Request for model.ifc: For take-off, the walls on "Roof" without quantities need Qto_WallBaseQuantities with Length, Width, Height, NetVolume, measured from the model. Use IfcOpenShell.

First a look at what the model holds.

```python
import ifcopenshell
import ifcopenshell.util.element
import ifcopenshell.util.unit

model = ifcopenshell.open("model.ifc")
print(model.schema)
for unit_type in ("LENGTHUNIT", "AREAUNIT", "VOLUMEUNIT"):
    print(unit_type, ifcopenshell.util.unit.calculate_unit_scale(model, unit_type))
storey = next(s for s in model.by_type("IfcBuildingStorey") if s.Name == "Roof")
walls = [e for e in ifcopenshell.util.element.get_decomposition(storey) if e.is_a("IfcWall")]
for e in sorted(walls, key=lambda e: e.id()):
    print(e.id(), e.is_a(), e.Name, list(ifcopenshell.util.element.get_psets(e, qtos_only=True)), sep=" | ")
```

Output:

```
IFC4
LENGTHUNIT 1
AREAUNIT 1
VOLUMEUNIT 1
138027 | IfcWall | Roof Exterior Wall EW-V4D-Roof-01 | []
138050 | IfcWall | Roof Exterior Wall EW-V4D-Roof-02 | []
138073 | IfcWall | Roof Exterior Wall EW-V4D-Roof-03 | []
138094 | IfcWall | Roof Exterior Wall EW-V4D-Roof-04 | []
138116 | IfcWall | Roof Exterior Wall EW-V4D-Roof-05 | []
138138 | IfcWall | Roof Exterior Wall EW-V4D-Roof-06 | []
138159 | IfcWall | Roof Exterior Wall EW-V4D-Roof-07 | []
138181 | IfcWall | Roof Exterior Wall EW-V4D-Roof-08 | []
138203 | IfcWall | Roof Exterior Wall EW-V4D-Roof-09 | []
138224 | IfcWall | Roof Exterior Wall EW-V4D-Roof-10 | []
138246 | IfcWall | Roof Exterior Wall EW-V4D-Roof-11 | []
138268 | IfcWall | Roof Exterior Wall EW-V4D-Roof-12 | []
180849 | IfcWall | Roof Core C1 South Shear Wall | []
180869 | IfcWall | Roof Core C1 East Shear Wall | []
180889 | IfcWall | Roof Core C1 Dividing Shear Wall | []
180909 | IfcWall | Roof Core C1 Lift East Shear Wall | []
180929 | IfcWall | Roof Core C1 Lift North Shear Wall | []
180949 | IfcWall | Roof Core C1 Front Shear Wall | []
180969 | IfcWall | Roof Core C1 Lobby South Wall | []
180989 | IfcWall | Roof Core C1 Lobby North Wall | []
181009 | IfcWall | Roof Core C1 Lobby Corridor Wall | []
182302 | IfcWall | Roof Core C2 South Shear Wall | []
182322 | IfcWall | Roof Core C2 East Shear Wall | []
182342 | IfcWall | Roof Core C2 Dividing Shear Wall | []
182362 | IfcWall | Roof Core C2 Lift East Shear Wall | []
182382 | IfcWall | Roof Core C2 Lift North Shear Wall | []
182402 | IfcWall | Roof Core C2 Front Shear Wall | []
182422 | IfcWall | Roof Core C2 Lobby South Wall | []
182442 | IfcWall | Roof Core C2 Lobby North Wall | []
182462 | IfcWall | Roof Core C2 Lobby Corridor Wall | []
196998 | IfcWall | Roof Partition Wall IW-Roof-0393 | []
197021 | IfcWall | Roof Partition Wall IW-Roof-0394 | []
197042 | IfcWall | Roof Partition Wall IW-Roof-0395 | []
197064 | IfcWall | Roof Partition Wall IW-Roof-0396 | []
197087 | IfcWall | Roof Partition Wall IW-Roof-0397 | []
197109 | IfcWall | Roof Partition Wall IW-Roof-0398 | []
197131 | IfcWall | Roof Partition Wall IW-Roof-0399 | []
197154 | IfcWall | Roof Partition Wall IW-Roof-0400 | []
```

```python
import ifcopenshell
import ifcopenshell.api.pset
import ifcopenshell.geom
import ifcopenshell.util.element
import ifcopenshell.util.shape
import ifcopenshell.util.unit

model = ifcopenshell.open("model.ifc")
unit_scale = ifcopenshell.util.unit.calculate_unit_scale(model)
volume_scale = ifcopenshell.util.unit.calculate_unit_scale(model, "VOLUMEUNIT")
settings = ifcopenshell.geom.settings()

storey = next(s for s in model.by_type("IfcBuildingStorey") if s.Name == "Roof")
walls = [e for e in ifcopenshell.util.element.get_decomposition(storey) if e.is_a("IfcWall")]

for e in sorted(walls, key=lambda e: e.id()):
    if ifcopenshell.util.element.get_psets(e, qtos_only=True, should_inherit=False):
        continue
    # Geometry comes back in metres, in the element's own axes.
    shape = ifcopenshell.geom.create_shape(settings, e)
    values = {
        "Length": ifcopenshell.util.shape.get_x(shape.geometry) / unit_scale,
        "Width": ifcopenshell.util.shape.get_y(shape.geometry) / unit_scale,
        "Height": ifcopenshell.util.shape.get_z(shape.geometry) / unit_scale,
        "NetVolume": ifcopenshell.util.shape.get_volume(shape.geometry) / volume_scale,
    }
    qto = ifcopenshell.api.pset.add_qto(model, product=e, name="Qto_WallBaseQuantities")
    ifcopenshell.api.pset.edit_qto(model, qto=qto, properties=values)
    print(e.id(), {k: round(v, 3) for k, v in values.items()})

model.write("model_v2.ifc")
```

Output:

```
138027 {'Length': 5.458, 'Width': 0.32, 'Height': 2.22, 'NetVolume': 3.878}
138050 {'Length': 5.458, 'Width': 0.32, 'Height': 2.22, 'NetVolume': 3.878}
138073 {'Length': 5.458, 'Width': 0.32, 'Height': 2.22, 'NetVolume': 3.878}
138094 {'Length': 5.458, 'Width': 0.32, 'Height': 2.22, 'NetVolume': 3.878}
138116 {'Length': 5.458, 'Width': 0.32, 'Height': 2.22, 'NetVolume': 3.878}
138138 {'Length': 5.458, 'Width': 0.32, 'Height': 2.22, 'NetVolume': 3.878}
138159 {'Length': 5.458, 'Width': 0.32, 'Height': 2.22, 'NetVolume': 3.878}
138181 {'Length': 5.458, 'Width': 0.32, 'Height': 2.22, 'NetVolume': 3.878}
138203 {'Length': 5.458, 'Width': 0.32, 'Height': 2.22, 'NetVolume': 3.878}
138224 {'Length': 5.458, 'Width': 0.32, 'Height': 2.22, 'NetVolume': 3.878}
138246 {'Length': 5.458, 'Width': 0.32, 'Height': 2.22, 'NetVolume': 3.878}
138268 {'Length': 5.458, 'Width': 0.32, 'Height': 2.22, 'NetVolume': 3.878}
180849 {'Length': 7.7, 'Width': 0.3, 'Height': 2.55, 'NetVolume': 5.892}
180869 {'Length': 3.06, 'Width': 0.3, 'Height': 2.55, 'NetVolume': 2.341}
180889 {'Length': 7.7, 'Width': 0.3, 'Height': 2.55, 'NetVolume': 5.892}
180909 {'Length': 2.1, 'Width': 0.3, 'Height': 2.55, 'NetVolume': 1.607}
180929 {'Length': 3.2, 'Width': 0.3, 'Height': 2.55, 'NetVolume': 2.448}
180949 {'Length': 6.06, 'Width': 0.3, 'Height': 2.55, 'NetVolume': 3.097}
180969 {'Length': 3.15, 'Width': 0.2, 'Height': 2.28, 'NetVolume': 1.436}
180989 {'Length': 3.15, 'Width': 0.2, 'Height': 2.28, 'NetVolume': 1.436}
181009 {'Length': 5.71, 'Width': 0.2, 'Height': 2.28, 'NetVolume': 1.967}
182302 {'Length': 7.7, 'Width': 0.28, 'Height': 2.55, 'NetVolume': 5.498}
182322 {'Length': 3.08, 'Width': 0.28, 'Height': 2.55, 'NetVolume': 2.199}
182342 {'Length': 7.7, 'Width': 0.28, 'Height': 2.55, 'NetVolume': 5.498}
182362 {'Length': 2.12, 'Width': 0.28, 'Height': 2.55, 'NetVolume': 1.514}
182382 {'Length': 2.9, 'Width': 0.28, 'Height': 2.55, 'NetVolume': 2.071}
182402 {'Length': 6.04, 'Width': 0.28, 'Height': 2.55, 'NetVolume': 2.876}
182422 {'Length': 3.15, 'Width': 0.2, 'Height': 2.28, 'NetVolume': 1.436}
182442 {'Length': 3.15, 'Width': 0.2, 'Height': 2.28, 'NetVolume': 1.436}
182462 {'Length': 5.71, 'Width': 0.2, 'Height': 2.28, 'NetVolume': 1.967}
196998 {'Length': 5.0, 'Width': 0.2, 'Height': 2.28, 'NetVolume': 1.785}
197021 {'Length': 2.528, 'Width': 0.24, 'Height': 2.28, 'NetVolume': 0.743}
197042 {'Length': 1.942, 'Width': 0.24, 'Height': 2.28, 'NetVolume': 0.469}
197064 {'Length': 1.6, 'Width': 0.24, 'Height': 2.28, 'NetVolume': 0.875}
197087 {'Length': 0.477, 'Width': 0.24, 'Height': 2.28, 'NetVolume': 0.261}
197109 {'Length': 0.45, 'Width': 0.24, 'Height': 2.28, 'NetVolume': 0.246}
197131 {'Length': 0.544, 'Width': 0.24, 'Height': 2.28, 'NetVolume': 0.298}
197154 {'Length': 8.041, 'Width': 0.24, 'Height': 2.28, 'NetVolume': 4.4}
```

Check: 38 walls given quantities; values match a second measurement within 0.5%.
